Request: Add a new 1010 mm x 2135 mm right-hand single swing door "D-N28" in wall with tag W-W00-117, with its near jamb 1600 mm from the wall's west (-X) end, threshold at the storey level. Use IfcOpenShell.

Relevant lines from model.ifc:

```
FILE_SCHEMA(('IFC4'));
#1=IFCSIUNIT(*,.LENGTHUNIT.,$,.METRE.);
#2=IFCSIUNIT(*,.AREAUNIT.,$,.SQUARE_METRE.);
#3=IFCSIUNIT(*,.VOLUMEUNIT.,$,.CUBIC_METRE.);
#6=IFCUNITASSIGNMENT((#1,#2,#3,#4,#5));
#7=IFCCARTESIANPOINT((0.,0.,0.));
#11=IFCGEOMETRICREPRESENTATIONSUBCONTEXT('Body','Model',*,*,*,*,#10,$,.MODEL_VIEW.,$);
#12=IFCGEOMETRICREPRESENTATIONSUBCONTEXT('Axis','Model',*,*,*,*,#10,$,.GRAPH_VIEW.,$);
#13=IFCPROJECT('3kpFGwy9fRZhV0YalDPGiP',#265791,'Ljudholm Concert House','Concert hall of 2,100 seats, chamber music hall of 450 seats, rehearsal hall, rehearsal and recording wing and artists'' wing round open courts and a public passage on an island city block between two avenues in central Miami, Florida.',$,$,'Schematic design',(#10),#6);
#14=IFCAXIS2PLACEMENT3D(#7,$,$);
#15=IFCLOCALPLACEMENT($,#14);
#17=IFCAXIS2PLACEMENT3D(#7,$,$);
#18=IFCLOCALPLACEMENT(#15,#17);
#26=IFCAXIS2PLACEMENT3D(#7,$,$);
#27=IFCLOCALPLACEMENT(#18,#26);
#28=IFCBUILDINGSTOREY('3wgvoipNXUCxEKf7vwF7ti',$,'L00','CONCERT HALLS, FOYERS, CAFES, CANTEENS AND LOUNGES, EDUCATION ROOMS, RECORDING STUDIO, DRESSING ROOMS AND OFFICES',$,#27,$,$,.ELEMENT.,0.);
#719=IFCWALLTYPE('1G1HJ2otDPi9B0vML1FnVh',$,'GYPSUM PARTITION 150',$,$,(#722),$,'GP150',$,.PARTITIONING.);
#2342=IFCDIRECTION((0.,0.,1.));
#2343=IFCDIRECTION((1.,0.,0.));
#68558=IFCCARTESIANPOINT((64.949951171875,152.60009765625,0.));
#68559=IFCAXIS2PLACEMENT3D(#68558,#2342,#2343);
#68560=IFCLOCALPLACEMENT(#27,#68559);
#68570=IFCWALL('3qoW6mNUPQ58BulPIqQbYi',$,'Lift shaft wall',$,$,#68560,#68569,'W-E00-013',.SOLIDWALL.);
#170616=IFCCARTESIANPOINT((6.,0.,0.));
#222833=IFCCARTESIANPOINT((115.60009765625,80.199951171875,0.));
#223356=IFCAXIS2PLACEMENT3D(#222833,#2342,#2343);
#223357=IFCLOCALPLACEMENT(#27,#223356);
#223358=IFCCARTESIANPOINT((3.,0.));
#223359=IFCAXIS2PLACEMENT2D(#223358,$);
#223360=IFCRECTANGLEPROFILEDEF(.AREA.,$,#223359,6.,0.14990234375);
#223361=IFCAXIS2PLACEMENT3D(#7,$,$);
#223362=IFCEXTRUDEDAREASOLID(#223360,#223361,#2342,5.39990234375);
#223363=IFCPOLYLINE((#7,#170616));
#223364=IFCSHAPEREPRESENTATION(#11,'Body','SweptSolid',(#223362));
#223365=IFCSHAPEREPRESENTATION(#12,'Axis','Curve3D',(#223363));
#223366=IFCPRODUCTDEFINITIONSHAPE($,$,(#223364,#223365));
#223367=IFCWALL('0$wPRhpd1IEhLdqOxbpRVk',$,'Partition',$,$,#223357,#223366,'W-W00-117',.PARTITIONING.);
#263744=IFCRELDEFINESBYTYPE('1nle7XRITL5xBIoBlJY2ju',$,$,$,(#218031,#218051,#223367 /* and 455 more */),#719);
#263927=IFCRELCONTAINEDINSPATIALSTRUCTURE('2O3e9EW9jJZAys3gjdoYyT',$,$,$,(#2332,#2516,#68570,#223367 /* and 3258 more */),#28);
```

```python
import numpy as np
import ifcopenshell
import ifcopenshell.api.feature
import ifcopenshell.api.geometry
import ifcopenshell.api.root
import ifcopenshell.api.spatial
import ifcopenshell.geom
import ifcopenshell.util.element
import ifcopenshell.util.placement
import ifcopenshell.util.representation
import ifcopenshell.util.shape
import ifcopenshell.util.unit

model = ifcopenshell.open("model.ifc")
unit_scale = ifcopenshell.util.unit.calculate_unit_scale(model)
settings = ifcopenshell.geom.settings()


def volume(element):
    """Net volume in cubic metres, openings subtracted."""
    shape = ifcopenshell.geom.create_shape(settings, element)
    return ifcopenshell.util.shape.get_volume(shape.geometry)


wall = model.by_guid("0$wPRhpd1IEhLdqOxbpRVk")
storey = ifcopenshell.util.element.get_container(wall, ifc_class="IfcBuildingStorey")
context = ifcopenshell.util.representation.get_context(model, "Model", "Body", "MODEL_VIEW")
before = volume(wall)

width, height, from_end, sill = 1.01, 2.135, 1.6, 0.0  # metres

# The wall runs along its own X axis, and the end named is its -X end.
wall_shape = ifcopenshell.geom.create_shape(settings, wall)
x, y, z = ifcopenshell.util.shape.get_vertices(wall_shape.geometry).T
start = x.min() + from_end
face, thickness = float(y.min()), float(y.max() - y.min())
wall_matrix = ifcopenshell.util.placement.get_local_placement(wall.ObjectPlacement)
level = ifcopenshell.util.placement.get_local_placement(storey.ObjectPlacement)[2, 3]


def in_wall(x, y):
    """Placement at x, y metres in the wall's axes, at sill height."""
    matrix = wall_matrix.copy()
    matrix[:, 3] = wall_matrix @ np.array([x / unit_scale, y / unit_scale, 0.0, 1.0])
    matrix[2, 3] = level + sill / unit_scale
    return matrix


# Opening: a box that overshoots both wall faces by 50 mm.
opening = ifcopenshell.api.root.create_entity(model, ifc_class="IfcOpeningElement", predefined_type="OPENING")
box = ifcopenshell.api.geometry.add_wall_representation(
    model, context=context, length=width, height=height, thickness=thickness + 0.1
)
ifcopenshell.api.geometry.assign_representation(model, product=opening, representation=box)
ifcopenshell.api.geometry.edit_object_placement(model, product=opening, matrix=in_wall(start, face - 0.05), is_si=False)
ifcopenshell.api.feature.add_feature(model, feature=opening, element=wall)

door = ifcopenshell.api.root.create_entity(model, ifc_class="IfcDoor", name="D-N28", predefined_type="DOOR")
door.OverallWidth, door.OverallHeight = width / unit_scale, height / unit_scale
door.OperationType = "SINGLE_SWING_RIGHT"
body = ifcopenshell.api.geometry.add_door_representation(
    model,
    context=context,
    overall_width=door.OverallWidth,
    overall_height=door.OverallHeight,
    operation_type="SINGLE_SWING_RIGHT",
    lining_properties={"LiningDepth": thickness / unit_scale, "ThresholdDepth": thickness / unit_scale},
)
ifcopenshell.api.geometry.assign_representation(model, product=door, representation=body)
ifcopenshell.api.spatial.assign_container(model, products=[door], relating_structure=storey)
ifcopenshell.api.feature.add_filling(model, opening=opening, element=door)

# The lining spans the wall, so the door starts at the wall face.
ifcopenshell.api.geometry.edit_object_placement(model, product=door, matrix=in_wall(start, face), is_si=False)

after = volume(wall)

print(f"wall volume {before:.3f} -> {after:.3f} m3")

model.write("model-out.ifc")
```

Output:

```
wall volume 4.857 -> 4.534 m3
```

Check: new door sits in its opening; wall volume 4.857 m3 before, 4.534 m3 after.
